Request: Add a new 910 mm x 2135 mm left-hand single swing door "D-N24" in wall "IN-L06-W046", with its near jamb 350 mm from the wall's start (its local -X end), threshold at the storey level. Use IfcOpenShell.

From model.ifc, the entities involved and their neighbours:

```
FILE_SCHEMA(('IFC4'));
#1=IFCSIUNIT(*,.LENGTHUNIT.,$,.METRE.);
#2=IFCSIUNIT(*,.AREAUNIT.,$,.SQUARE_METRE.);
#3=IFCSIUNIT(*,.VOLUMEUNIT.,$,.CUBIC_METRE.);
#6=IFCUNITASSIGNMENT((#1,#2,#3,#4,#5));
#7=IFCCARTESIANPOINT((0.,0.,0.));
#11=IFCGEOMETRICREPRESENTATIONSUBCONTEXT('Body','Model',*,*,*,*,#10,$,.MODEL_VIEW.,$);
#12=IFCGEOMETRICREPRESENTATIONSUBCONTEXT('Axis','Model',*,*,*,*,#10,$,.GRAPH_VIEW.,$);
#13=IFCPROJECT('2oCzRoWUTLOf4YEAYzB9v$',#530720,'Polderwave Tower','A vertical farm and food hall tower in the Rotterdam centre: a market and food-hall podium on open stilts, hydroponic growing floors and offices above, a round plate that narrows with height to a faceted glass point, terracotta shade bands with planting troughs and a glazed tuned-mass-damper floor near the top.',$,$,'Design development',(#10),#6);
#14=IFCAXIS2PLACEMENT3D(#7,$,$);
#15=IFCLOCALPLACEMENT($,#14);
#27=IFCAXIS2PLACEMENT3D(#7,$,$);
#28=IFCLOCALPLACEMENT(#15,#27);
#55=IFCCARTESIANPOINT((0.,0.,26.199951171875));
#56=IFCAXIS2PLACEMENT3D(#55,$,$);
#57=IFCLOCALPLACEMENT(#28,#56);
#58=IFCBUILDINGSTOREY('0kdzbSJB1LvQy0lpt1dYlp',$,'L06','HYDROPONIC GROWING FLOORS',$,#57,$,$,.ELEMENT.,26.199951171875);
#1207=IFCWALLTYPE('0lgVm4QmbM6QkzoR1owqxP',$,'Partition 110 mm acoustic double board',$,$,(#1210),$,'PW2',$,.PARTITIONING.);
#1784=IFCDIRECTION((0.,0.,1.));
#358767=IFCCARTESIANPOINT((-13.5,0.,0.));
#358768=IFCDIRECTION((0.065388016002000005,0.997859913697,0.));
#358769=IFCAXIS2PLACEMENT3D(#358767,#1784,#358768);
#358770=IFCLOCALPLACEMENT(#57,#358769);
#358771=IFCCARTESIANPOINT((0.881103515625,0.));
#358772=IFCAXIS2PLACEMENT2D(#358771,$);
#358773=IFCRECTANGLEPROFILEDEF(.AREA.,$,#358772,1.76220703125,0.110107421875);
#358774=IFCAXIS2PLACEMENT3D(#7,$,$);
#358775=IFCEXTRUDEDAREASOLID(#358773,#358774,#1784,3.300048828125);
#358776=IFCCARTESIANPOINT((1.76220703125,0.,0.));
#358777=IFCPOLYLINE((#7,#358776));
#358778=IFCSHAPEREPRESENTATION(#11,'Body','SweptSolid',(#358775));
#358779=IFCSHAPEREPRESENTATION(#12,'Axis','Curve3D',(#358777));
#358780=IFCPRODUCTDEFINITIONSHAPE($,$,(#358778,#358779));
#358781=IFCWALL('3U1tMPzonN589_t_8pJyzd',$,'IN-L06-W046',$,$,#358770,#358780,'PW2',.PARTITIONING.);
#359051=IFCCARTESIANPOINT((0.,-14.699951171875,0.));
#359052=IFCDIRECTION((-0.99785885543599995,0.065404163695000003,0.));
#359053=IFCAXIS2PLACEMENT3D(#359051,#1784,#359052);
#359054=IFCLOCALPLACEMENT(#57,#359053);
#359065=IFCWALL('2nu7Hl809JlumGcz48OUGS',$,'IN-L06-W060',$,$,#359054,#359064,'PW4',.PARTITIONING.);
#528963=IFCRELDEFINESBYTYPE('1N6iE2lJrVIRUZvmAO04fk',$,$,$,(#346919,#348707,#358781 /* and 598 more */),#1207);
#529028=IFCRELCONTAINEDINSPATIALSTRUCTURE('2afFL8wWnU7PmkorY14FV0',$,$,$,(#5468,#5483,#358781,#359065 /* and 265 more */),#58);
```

```python
import numpy as np
import ifcopenshell
import ifcopenshell.api.feature
import ifcopenshell.api.geometry
import ifcopenshell.api.root
import ifcopenshell.api.spatial
import ifcopenshell.geom
import ifcopenshell.util.element
import ifcopenshell.util.placement
import ifcopenshell.util.representation
import ifcopenshell.util.shape
import ifcopenshell.util.unit

model = ifcopenshell.open("model.ifc")
unit_scale = ifcopenshell.util.unit.calculate_unit_scale(model)
settings = ifcopenshell.geom.settings()


def volume(element):
    """Net volume in cubic metres, openings subtracted."""
    shape = ifcopenshell.geom.create_shape(settings, element)
    return ifcopenshell.util.shape.get_volume(shape.geometry)


wall = model.by_guid("3U1tMPzonN589_t_8pJyzd")
storey = ifcopenshell.util.element.get_container(wall, ifc_class="IfcBuildingStorey")
context = ifcopenshell.util.representation.get_context(model, "Model", "Body", "MODEL_VIEW")
before = volume(wall)

width, height, from_end, sill = 0.91, 2.135, 0.35, 0.0  # metres

# The wall runs along its own X axis, and the end named is its -X end.
wall_shape = ifcopenshell.geom.create_shape(settings, wall)
x, y, z = ifcopenshell.util.shape.get_vertices(wall_shape.geometry).T
start = x.min() + from_end
face, thickness = float(y.min()), float(y.max() - y.min())
wall_matrix = ifcopenshell.util.placement.get_local_placement(wall.ObjectPlacement)
level = ifcopenshell.util.placement.get_local_placement(storey.ObjectPlacement)[2, 3]


def in_wall(x, y):
    """Placement at x, y metres in the wall's axes, at sill height."""
    matrix = wall_matrix.copy()
    matrix[:, 3] = wall_matrix @ np.array([x / unit_scale, y / unit_scale, 0.0, 1.0])
    matrix[2, 3] = level + sill / unit_scale
    return matrix


# Opening: a box that overshoots both wall faces by 50 mm.
opening = ifcopenshell.api.root.create_entity(model, ifc_class="IfcOpeningElement", predefined_type="OPENING")
box = ifcopenshell.api.geometry.add_wall_representation(
    model, context=context, length=width, height=height, thickness=thickness + 0.1
)
ifcopenshell.api.geometry.assign_representation(model, product=opening, representation=box)
ifcopenshell.api.geometry.edit_object_placement(model, product=opening, matrix=in_wall(start, face - 0.05), is_si=False)
ifcopenshell.api.feature.add_feature(model, feature=opening, element=wall)

door = ifcopenshell.api.root.create_entity(model, ifc_class="IfcDoor", name="D-N24", predefined_type="DOOR")
door.OverallWidth, door.OverallHeight = width / unit_scale, height / unit_scale
door.OperationType = "SINGLE_SWING_LEFT"
body = ifcopenshell.api.geometry.add_door_representation(
    model,
    context=context,
    overall_width=door.OverallWidth,
    overall_height=door.OverallHeight,
    operation_type="SINGLE_SWING_LEFT",
    lining_properties={"LiningDepth": thickness / unit_scale, "ThresholdDepth": thickness / unit_scale},
)
ifcopenshell.api.geometry.assign_representation(model, product=door, representation=body)
ifcopenshell.api.spatial.assign_container(model, products=[door], relating_structure=storey)
ifcopenshell.api.feature.add_filling(model, opening=opening, element=door)

# The lining spans the wall, so the door starts at the wall face.
ifcopenshell.api.geometry.edit_object_placement(model, product=door, matrix=in_wall(start, face), is_si=False)

after = volume(wall)

print(f"wall volume {before:.3f} -> {after:.3f} m3")

model.write("model_edited.ifc")
```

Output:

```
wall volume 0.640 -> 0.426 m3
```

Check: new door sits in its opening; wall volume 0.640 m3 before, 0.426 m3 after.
